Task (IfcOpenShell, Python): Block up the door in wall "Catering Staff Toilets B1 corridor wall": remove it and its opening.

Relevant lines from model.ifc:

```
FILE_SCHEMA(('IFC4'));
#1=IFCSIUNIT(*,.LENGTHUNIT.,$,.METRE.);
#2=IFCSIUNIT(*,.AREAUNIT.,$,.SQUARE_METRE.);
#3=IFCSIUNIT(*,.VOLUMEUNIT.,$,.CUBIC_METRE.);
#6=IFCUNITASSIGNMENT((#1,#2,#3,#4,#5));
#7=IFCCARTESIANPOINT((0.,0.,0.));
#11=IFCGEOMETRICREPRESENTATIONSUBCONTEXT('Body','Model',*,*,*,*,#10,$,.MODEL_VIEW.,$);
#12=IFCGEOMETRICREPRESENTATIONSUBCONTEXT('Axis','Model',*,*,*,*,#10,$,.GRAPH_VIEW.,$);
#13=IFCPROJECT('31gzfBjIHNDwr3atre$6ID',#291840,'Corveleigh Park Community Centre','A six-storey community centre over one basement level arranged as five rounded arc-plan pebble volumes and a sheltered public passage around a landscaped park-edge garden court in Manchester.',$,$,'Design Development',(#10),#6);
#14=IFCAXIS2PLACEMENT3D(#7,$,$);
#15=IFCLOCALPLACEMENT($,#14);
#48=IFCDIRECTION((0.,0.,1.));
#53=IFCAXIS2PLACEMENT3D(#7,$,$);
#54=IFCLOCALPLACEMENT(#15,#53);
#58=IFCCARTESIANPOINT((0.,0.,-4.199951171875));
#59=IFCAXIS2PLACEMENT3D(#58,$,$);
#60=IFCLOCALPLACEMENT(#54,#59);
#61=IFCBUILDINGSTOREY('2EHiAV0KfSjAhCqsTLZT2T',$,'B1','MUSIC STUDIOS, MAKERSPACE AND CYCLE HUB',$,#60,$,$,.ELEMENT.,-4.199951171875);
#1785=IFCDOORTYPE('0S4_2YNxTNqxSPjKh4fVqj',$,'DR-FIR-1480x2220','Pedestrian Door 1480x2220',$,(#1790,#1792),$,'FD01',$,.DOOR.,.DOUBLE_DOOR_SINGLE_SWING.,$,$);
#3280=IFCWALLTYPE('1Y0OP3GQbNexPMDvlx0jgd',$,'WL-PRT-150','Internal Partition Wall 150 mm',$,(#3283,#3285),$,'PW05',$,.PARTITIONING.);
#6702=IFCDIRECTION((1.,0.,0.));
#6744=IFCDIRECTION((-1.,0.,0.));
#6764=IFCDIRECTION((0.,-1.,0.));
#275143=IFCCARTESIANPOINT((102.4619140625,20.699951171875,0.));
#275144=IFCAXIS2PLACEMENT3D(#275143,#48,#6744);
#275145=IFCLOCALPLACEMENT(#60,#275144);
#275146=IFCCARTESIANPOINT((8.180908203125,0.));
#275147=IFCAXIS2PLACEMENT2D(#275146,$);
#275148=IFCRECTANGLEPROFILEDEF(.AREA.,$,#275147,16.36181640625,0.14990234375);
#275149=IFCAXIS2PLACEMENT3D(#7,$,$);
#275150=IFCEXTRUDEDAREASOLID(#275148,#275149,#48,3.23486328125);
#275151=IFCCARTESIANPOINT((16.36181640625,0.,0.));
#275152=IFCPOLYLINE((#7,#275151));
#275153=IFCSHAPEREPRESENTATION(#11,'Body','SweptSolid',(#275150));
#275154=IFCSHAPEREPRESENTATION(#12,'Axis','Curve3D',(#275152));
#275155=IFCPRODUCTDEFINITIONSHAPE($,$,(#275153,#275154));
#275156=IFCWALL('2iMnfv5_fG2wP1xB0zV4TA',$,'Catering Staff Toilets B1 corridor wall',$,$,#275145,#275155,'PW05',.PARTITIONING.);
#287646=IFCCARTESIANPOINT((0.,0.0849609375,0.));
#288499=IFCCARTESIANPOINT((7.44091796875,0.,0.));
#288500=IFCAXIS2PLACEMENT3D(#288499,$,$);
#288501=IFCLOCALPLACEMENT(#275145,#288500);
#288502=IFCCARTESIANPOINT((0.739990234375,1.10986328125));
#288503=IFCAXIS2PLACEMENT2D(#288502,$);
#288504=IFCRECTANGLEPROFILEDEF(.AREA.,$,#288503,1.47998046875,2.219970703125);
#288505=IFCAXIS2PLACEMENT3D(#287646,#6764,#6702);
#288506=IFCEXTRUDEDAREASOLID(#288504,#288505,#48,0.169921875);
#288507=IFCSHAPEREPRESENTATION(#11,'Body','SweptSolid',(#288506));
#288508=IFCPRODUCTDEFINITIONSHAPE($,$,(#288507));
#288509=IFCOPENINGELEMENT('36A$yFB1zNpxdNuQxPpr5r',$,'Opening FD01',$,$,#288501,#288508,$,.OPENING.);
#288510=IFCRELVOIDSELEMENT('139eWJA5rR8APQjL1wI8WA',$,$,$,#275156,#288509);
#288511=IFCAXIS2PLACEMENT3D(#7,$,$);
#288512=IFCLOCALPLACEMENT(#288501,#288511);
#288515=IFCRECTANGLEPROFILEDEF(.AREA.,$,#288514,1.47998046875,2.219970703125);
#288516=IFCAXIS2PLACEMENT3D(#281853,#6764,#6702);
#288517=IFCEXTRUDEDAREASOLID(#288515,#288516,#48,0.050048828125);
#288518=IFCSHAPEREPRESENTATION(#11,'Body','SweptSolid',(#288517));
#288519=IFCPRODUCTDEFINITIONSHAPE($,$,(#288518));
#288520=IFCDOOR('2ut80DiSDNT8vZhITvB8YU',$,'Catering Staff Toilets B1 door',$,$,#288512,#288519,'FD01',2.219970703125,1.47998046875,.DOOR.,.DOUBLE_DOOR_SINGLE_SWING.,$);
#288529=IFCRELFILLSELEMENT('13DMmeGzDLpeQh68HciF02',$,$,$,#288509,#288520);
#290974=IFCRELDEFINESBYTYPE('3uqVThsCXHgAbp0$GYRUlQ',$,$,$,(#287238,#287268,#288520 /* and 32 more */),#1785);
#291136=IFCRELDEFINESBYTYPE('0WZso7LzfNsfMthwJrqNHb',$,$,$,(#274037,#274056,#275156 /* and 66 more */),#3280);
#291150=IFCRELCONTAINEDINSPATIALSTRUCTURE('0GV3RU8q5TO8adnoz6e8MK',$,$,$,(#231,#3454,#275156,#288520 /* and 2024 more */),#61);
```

```python
import ifcopenshell
import ifcopenshell.api.feature
import ifcopenshell.api.root
import ifcopenshell.geom
import ifcopenshell.util.shape

model = ifcopenshell.open("model.ifc")
settings = ifcopenshell.geom.settings()


def volume(element):
    """Net volume in cubic metres, openings subtracted."""
    shape = ifcopenshell.geom.create_shape(settings, element)
    return ifcopenshell.util.shape.get_volume(shape.geometry)


door = model.by_guid("2ut80DiSDNT8vZhITvB8YU")
opening = door.FillsVoids[0].RelatingOpeningElement
wall = opening.VoidsElements[0].RelatingBuildingElement
before = volume(wall)

ifcopenshell.api.root.remove_product(model, product=door)
ifcopenshell.api.feature.remove_feature(model, feature=opening)

after = volume(wall)

print(f"wall volume {before:.3f} -> {after:.3f} m3")

model.write("model_edited.ifc")
```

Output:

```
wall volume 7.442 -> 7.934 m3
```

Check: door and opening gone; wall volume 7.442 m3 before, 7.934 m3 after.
